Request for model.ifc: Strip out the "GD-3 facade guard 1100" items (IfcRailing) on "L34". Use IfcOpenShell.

First a look at what the model holds.

```python
import ifcopenshell
import ifcopenshell.util.element

model = ifcopenshell.open("model.ifc")
print(model.schema)
storey = next(s for s in model.by_type("IfcBuildingStorey") if s.Name == "L34")
railings = [e for e in ifcopenshell.util.element.get_decomposition(storey) if e.is_a("IfcRailing")]
seen = {}
for e in railings:
    element_type = ifcopenshell.util.element.get_type(e)
    name = element_type.Name if element_type not in (None, e) else None
    seen[name] = seen.get(name, 0) + 1
for name, count in sorted(seen.items(), key=str):
    print(count, "x", name)
```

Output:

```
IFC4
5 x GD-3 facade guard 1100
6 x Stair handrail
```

```python
import ifcopenshell
import ifcopenshell.api.root
import ifcopenshell.util.element

model = ifcopenshell.open("model.ifc")

storey = next(s for s in model.by_type("IfcBuildingStorey") if s.Name == "L34")
railings = [e for e in ifcopenshell.util.element.get_decomposition(storey) if e.is_a("IfcRailing")]
targets = [e for e in railings if (t := ifcopenshell.util.element.get_type(e)) not in (None, e) and t.Name == "GD-3 facade guard 1100"]

for e in targets:
    ifcopenshell.api.root.remove_product(model, product=e)
print(len(targets), "removed")

model.write("model_v2.ifc")
```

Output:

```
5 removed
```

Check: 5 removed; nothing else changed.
